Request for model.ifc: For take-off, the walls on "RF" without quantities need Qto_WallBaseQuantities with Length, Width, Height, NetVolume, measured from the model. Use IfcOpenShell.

First a look at what the model holds.

```python
import ifcopenshell
import ifcopenshell.util.element
import ifcopenshell.util.unit

model = ifcopenshell.open("model.ifc")
print(model.schema)
for unit_type in ("LENGTHUNIT", "AREAUNIT", "VOLUMEUNIT"):
    print(unit_type, ifcopenshell.util.unit.calculate_unit_scale(model, unit_type))
storey = next(s for s in model.by_type("IfcBuildingStorey") if s.Name == "RF")
walls = [e for e in ifcopenshell.util.element.get_decomposition(storey) if e.is_a("IfcWall")]
for e in sorted(walls, key=lambda e: e.id()):
    print(e.id(), e.is_a(), e.Name, list(ifcopenshell.util.element.get_psets(e, qtos_only=True)), sep=" | ")
```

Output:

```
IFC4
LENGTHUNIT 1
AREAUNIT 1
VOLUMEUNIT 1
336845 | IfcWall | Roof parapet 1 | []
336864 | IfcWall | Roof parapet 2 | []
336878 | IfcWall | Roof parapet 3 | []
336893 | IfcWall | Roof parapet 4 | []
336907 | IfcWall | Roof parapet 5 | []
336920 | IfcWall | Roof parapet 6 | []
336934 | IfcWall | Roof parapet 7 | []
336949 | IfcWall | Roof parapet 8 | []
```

```python
import ifcopenshell
import ifcopenshell.api.pset
import ifcopenshell.geom
import ifcopenshell.util.element
import ifcopenshell.util.shape
import ifcopenshell.util.unit

model = ifcopenshell.open("model.ifc")
unit_scale = ifcopenshell.util.unit.calculate_unit_scale(model)
volume_scale = ifcopenshell.util.unit.calculate_unit_scale(model, "VOLUMEUNIT")
settings = ifcopenshell.geom.settings()

storey = next(s for s in model.by_type("IfcBuildingStorey") if s.Name == "RF")
walls = [e for e in ifcopenshell.util.element.get_decomposition(storey) if e.is_a("IfcWall")]

for e in sorted(walls, key=lambda e: e.id()):
    if ifcopenshell.util.element.get_psets(e, qtos_only=True, should_inherit=False):
        continue
    # Geometry comes back in metres, in the element's own axes.
    shape = ifcopenshell.geom.create_shape(settings, e)
    values = {
        "Length": ifcopenshell.util.shape.get_x(shape.geometry) / unit_scale,
        "Width": ifcopenshell.util.shape.get_y(shape.geometry) / unit_scale,
        "Height": ifcopenshell.util.shape.get_z(shape.geometry) / unit_scale,
        "NetVolume": ifcopenshell.util.shape.get_volume(shape.geometry) / volume_scale,
    }
    qto = ifcopenshell.api.pset.add_qto(model, product=e, name="Qto_WallBaseQuantities")
    ifcopenshell.api.pset.edit_qto(model, qto=qto, properties=values)
    print(e.id(), {k: round(v, 3) for k, v in values.items()})

model.write("model-out.ifc")
```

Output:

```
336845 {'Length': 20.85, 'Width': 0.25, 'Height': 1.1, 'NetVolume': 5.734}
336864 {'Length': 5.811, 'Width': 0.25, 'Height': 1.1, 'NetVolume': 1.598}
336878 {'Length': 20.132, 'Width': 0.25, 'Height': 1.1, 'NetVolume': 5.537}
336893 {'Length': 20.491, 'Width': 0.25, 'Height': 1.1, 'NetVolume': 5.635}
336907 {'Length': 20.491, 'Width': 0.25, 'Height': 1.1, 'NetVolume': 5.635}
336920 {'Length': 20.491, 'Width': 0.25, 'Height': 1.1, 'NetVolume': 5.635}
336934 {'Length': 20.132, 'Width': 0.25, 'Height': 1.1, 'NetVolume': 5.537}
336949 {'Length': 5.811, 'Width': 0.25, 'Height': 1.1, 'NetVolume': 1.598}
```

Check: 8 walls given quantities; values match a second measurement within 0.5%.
